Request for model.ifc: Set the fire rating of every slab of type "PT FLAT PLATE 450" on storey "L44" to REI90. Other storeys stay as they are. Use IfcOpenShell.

First a look at what the model holds.

```python
import ifcopenshell
import ifcopenshell.util.element

model = ifcopenshell.open("model.ifc")
print(model.schema)
storey = next(s for s in model.by_type("IfcBuildingStorey") if s.Name == "L44")
slabs = [e for e in ifcopenshell.util.element.get_decomposition(storey) if e.is_a("IfcSlab")]
seen = {}
for e in slabs:
    element_type = ifcopenshell.util.element.get_type(e)
    key = (element_type.Name if element_type != e and element_type else None, ifcopenshell.util.element.get_pset(e, "Pset_SlabCommon", "FireRating"))
    seen[key] = seen.get(key, 0) + 1
for (name, value), count in sorted(seen.items(), key=str):
    print(count, "x", name, "|", value)
```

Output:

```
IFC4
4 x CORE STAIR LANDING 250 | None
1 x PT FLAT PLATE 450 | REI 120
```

```python
import ifcopenshell
import ifcopenshell.api.pset
import ifcopenshell.util.element

model = ifcopenshell.open("model.ifc")

storey = next(s for s in model.by_type("IfcBuildingStorey") if s.Name == "L44")
slabs = [e for e in ifcopenshell.util.element.get_decomposition(storey) if e.is_a("IfcSlab")]

count = 0
for e in slabs:
    element_type = ifcopenshell.util.element.get_type(e)
    if element_type in (None, e) or element_type.Name != "PT FLAT PLATE 450":
        continue
    found = ifcopenshell.util.element.get_pset(e, "Pset_SlabCommon", should_inherit=False)
    if found:
        pset = model.by_id(found["id"])
        if len(ifcopenshell.util.element.get_elements_by_pset(pset)) > 1:
            pset = ifcopenshell.api.pset.unshare_pset(model, products=[e], pset=pset)[0]
    else:
        pset = ifcopenshell.api.pset.add_pset(model, product=e, name="Pset_SlabCommon")
    ifcopenshell.api.pset.edit_pset(model, pset=pset, properties={"FireRating": "REI90"})
    count += 1

print(count, "slabs updated")

model.write("model_rev.ifc")
```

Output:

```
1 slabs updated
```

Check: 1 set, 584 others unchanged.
